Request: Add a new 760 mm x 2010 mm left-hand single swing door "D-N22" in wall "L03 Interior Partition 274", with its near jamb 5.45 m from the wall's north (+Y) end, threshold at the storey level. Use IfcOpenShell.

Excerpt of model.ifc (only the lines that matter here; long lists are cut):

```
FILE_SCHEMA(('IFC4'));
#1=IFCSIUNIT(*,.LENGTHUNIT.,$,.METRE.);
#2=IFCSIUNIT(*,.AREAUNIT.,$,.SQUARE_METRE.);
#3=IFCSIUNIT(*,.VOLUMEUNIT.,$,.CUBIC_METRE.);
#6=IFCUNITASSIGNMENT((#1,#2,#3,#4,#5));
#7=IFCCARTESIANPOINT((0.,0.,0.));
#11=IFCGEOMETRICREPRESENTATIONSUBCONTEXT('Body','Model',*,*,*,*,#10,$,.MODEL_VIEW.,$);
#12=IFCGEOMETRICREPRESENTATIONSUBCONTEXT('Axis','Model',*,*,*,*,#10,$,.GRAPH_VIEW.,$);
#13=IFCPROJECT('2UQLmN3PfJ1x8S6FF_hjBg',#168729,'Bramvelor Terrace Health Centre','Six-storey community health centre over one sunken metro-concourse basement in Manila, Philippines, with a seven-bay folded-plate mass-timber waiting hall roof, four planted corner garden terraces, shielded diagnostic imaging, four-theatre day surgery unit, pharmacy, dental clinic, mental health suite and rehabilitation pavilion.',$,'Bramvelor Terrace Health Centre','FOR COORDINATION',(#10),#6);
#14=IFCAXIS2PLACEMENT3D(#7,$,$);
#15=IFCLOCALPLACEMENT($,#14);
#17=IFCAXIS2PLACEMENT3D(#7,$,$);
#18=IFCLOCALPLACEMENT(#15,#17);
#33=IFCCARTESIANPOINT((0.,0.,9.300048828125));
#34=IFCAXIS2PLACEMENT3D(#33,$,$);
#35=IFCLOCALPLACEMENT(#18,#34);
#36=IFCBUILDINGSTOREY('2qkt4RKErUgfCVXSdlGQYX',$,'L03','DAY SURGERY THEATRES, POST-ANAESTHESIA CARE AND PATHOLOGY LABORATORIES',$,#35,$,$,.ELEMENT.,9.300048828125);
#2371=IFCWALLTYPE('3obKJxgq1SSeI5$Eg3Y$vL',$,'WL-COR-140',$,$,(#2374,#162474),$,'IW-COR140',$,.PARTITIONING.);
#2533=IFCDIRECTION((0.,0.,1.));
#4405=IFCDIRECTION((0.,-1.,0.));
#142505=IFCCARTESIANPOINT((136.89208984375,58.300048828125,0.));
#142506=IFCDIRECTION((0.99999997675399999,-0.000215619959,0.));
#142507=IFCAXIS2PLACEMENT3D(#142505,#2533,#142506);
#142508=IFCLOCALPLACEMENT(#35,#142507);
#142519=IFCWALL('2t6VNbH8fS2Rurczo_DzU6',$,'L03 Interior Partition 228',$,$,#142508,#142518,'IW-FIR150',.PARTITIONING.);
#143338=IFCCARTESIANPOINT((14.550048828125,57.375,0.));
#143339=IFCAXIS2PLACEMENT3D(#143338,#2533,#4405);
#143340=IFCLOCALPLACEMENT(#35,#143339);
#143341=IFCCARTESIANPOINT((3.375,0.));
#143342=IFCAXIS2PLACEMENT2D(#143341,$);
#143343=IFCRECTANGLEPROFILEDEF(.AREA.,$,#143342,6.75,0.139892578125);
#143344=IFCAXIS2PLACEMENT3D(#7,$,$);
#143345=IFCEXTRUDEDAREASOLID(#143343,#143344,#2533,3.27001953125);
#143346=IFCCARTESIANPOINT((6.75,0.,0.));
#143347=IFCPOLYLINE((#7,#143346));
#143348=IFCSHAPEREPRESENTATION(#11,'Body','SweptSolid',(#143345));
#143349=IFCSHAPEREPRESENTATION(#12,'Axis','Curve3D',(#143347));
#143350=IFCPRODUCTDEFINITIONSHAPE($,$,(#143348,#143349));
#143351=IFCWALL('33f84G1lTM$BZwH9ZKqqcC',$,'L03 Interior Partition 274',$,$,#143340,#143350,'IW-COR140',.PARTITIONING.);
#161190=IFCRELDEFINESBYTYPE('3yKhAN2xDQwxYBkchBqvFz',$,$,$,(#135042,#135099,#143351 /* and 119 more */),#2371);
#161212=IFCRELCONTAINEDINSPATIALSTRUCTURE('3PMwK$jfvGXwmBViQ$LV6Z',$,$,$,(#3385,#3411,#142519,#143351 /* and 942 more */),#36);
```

```python
import numpy as np
import ifcopenshell
import ifcopenshell.api.feature
import ifcopenshell.api.geometry
import ifcopenshell.api.root
import ifcopenshell.api.spatial
import ifcopenshell.geom
import ifcopenshell.util.element
import ifcopenshell.util.placement
import ifcopenshell.util.representation
import ifcopenshell.util.shape
import ifcopenshell.util.unit

model = ifcopenshell.open("model.ifc")
unit_scale = ifcopenshell.util.unit.calculate_unit_scale(model)
settings = ifcopenshell.geom.settings()


def volume(element):
    """Net volume in cubic metres, openings subtracted."""
    shape = ifcopenshell.geom.create_shape(settings, element)
    return ifcopenshell.util.shape.get_volume(shape.geometry)


wall = model.by_guid("33f84G1lTM$BZwH9ZKqqcC")
storey = ifcopenshell.util.element.get_container(wall, ifc_class="IfcBuildingStorey")
context = ifcopenshell.util.representation.get_context(model, "Model", "Body", "MODEL_VIEW")
before = volume(wall)

width, height, from_end, sill = 0.76, 2.01, 5.45, 0.0  # metres

# The wall runs along its own X axis, and the end named is its -X end.
wall_shape = ifcopenshell.geom.create_shape(settings, wall)
x, y, z = ifcopenshell.util.shape.get_vertices(wall_shape.geometry).T
start = x.min() + from_end
face, thickness = float(y.min()), float(y.max() - y.min())
wall_matrix = ifcopenshell.util.placement.get_local_placement(wall.ObjectPlacement)
level = ifcopenshell.util.placement.get_local_placement(storey.ObjectPlacement)[2, 3]


def in_wall(x, y):
    """Placement at x, y metres in the wall's axes, at sill height."""
    matrix = wall_matrix.copy()
    matrix[:, 3] = wall_matrix @ np.array([x / unit_scale, y / unit_scale, 0.0, 1.0])
    matrix[2, 3] = level + sill / unit_scale
    return matrix


# Opening: a box that overshoots both wall faces by 50 mm.
opening = ifcopenshell.api.root.create_entity(model, ifc_class="IfcOpeningElement", predefined_type="OPENING")
box = ifcopenshell.api.geometry.add_wall_representation(
    model, context=context, length=width, height=height, thickness=thickness + 0.1
)
ifcopenshell.api.geometry.assign_representation(model, product=opening, representation=box)
ifcopenshell.api.geometry.edit_object_placement(model, product=opening, matrix=in_wall(start, face - 0.05), is_si=False)
ifcopenshell.api.feature.add_feature(model, feature=opening, element=wall)

door = ifcopenshell.api.root.create_entity(model, ifc_class="IfcDoor", name="D-N22", predefined_type="DOOR")
door.OverallWidth, door.OverallHeight = width / unit_scale, height / unit_scale
door.OperationType = "SINGLE_SWING_LEFT"
body = ifcopenshell.api.geometry.add_door_representation(
    model,
    context=context,
    overall_width=door.OverallWidth,
    overall_height=door.OverallHeight,
    operation_type="SINGLE_SWING_LEFT",
    lining_properties={"LiningDepth": thickness / unit_scale, "ThresholdDepth": thickness / unit_scale},
)
ifcopenshell.api.geometry.assign_representation(model, product=door, representation=body)
ifcopenshell.api.spatial.assign_container(model, products=[door], relating_structure=storey)
ifcopenshell.api.feature.add_filling(model, opening=opening, element=door)

# The lining spans the wall, so the door starts at the wall face.
ifcopenshell.api.geometry.edit_object_placement(model, product=door, matrix=in_wall(start, face), is_si=False)

after = volume(wall)

print(f"wall volume {before:.3f} -> {after:.3f} m3")

model.write("model_v2.ifc")
```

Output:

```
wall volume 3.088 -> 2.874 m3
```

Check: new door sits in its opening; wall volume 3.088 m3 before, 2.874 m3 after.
